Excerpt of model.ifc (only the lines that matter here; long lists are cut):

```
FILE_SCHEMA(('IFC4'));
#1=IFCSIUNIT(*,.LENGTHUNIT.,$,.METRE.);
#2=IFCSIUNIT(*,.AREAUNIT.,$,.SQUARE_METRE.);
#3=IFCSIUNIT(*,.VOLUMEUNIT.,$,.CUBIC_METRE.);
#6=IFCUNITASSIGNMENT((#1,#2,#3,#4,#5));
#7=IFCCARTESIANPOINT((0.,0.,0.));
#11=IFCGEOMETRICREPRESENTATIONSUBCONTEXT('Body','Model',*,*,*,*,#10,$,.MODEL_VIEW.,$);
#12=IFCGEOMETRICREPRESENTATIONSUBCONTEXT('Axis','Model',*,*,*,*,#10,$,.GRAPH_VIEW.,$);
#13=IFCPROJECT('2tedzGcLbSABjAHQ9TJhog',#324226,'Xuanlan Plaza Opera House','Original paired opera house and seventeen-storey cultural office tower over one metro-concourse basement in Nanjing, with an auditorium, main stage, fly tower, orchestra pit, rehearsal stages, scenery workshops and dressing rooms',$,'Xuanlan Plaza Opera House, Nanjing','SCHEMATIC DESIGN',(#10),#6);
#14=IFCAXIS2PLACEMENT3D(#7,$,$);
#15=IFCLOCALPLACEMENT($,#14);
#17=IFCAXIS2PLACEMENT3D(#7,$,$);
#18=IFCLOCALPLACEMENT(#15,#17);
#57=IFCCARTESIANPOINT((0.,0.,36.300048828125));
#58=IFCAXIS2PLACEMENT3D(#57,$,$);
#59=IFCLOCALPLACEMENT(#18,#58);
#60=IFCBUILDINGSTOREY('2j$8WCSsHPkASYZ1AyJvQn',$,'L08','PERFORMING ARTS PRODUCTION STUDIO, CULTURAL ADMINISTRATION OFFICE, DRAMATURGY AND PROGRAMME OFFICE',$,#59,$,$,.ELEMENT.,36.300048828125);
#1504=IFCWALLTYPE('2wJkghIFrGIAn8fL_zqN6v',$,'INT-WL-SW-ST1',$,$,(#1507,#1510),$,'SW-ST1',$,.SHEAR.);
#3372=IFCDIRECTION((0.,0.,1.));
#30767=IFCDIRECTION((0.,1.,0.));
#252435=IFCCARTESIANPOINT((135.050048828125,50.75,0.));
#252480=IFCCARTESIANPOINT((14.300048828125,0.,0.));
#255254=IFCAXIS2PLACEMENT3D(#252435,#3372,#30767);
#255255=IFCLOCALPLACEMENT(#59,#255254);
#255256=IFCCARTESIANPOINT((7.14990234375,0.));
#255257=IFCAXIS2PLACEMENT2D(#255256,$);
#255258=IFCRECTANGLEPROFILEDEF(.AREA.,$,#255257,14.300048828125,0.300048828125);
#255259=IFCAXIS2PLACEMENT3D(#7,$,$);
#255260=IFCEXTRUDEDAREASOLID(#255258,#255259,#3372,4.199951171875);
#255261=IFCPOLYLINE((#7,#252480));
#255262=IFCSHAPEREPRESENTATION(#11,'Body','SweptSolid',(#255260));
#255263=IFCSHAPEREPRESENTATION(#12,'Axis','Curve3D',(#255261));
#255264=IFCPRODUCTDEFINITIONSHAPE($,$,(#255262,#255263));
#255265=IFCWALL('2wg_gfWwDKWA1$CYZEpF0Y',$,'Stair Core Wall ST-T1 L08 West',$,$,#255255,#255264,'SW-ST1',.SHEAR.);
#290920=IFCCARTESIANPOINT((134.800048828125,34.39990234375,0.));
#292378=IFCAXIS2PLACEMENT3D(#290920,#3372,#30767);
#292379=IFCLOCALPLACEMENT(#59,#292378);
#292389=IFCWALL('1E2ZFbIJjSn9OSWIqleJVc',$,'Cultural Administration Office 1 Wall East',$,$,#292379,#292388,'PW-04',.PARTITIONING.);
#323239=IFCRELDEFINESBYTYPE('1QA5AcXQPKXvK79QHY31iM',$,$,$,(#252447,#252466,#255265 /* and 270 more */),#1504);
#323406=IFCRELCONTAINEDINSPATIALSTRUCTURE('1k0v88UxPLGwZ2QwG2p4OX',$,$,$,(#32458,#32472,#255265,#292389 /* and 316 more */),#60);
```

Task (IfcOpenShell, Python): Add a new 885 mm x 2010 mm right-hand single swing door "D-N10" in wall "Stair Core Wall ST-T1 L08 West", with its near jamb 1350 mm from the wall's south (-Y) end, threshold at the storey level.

```python
import numpy as np
import ifcopenshell
import ifcopenshell.api.feature
import ifcopenshell.api.geometry
import ifcopenshell.api.root
import ifcopenshell.api.spatial
import ifcopenshell.geom
import ifcopenshell.util.element
import ifcopenshell.util.placement
import ifcopenshell.util.representation
import ifcopenshell.util.shape
import ifcopenshell.util.unit

model = ifcopenshell.open("model.ifc")
unit_scale = ifcopenshell.util.unit.calculate_unit_scale(model)
settings = ifcopenshell.geom.settings()


def volume(element):
    """Net volume in cubic metres, openings subtracted."""
    shape = ifcopenshell.geom.create_shape(settings, element)
    return ifcopenshell.util.shape.get_volume(shape.geometry)


wall = model.by_id(255265)
storey = ifcopenshell.util.element.get_container(wall, ifc_class="IfcBuildingStorey")
context = ifcopenshell.util.representation.get_context(model, "Model", "Body", "MODEL_VIEW")
before = volume(wall)

width, height, from_end, sill = 0.885, 2.01, 1.35, 0.0  # metres

# The wall runs along its own X axis, and the end named is its -X end.
wall_shape = ifcopenshell.geom.create_shape(settings, wall)
x, y, z = ifcopenshell.util.shape.get_vertices(wall_shape.geometry).T
start = x.min() + from_end
face, thickness = float(y.min()), float(y.max() - y.min())
wall_matrix = ifcopenshell.util.placement.get_local_placement(wall.ObjectPlacement)
level = ifcopenshell.util.placement.get_local_placement(storey.ObjectPlacement)[2, 3]


def in_wall(x, y):
    """Placement at x, y metres in the wall's axes, at sill height."""
    matrix = wall_matrix.copy()
    matrix[:, 3] = wall_matrix @ np.array([x / unit_scale, y / unit_scale, 0.0, 1.0])
    matrix[2, 3] = level + sill / unit_scale
    return matrix


# Opening: a box that overshoots both wall faces by 50 mm.
opening = ifcopenshell.api.root.create_entity(model, ifc_class="IfcOpeningElement", predefined_type="OPENING")
box = ifcopenshell.api.geometry.add_wall_representation(
    model, context=context, length=width, height=height, thickness=thickness + 0.1
)
ifcopenshell.api.geometry.assign_representation(model, product=opening, representation=box)
ifcopenshell.api.geometry.edit_object_placement(model, product=opening, matrix=in_wall(start, face - 0.05), is_si=False)
ifcopenshell.api.feature.add_feature(model, feature=opening, element=wall)

door = ifcopenshell.api.root.create_entity(model, ifc_class="IfcDoor", name="D-N10", predefined_type="DOOR")
door.OverallWidth, door.OverallHeight = width / unit_scale, height / unit_scale
door.OperationType = "SINGLE_SWING_RIGHT"
body = ifcopenshell.api.geometry.add_door_representation(
    model,
    context=context,
    overall_width=door.OverallWidth,
    overall_height=door.OverallHeight,
    operation_type="SINGLE_SWING_RIGHT",
    lining_properties={"LiningDepth": thickness / unit_scale, "ThresholdDepth": thickness / unit_scale},
)
ifcopenshell.api.geometry.assign_representation(model, product=door, representation=body)
ifcopenshell.api.spatial.assign_container(model, products=[door], relating_structure=storey)
ifcopenshell.api.feature.add_filling(model, opening=opening, element=door)

# The lining spans the wall, so the door starts at the wall face.
ifcopenshell.api.geometry.edit_object_placement(model, product=door, matrix=in_wall(start, face), is_si=False)

after = volume(wall)

print(f"wall volume {before:.3f} -> {after:.3f} m3")

model.write("model_rev.ifc")
```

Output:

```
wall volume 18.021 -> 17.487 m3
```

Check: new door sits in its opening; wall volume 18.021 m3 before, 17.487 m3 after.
